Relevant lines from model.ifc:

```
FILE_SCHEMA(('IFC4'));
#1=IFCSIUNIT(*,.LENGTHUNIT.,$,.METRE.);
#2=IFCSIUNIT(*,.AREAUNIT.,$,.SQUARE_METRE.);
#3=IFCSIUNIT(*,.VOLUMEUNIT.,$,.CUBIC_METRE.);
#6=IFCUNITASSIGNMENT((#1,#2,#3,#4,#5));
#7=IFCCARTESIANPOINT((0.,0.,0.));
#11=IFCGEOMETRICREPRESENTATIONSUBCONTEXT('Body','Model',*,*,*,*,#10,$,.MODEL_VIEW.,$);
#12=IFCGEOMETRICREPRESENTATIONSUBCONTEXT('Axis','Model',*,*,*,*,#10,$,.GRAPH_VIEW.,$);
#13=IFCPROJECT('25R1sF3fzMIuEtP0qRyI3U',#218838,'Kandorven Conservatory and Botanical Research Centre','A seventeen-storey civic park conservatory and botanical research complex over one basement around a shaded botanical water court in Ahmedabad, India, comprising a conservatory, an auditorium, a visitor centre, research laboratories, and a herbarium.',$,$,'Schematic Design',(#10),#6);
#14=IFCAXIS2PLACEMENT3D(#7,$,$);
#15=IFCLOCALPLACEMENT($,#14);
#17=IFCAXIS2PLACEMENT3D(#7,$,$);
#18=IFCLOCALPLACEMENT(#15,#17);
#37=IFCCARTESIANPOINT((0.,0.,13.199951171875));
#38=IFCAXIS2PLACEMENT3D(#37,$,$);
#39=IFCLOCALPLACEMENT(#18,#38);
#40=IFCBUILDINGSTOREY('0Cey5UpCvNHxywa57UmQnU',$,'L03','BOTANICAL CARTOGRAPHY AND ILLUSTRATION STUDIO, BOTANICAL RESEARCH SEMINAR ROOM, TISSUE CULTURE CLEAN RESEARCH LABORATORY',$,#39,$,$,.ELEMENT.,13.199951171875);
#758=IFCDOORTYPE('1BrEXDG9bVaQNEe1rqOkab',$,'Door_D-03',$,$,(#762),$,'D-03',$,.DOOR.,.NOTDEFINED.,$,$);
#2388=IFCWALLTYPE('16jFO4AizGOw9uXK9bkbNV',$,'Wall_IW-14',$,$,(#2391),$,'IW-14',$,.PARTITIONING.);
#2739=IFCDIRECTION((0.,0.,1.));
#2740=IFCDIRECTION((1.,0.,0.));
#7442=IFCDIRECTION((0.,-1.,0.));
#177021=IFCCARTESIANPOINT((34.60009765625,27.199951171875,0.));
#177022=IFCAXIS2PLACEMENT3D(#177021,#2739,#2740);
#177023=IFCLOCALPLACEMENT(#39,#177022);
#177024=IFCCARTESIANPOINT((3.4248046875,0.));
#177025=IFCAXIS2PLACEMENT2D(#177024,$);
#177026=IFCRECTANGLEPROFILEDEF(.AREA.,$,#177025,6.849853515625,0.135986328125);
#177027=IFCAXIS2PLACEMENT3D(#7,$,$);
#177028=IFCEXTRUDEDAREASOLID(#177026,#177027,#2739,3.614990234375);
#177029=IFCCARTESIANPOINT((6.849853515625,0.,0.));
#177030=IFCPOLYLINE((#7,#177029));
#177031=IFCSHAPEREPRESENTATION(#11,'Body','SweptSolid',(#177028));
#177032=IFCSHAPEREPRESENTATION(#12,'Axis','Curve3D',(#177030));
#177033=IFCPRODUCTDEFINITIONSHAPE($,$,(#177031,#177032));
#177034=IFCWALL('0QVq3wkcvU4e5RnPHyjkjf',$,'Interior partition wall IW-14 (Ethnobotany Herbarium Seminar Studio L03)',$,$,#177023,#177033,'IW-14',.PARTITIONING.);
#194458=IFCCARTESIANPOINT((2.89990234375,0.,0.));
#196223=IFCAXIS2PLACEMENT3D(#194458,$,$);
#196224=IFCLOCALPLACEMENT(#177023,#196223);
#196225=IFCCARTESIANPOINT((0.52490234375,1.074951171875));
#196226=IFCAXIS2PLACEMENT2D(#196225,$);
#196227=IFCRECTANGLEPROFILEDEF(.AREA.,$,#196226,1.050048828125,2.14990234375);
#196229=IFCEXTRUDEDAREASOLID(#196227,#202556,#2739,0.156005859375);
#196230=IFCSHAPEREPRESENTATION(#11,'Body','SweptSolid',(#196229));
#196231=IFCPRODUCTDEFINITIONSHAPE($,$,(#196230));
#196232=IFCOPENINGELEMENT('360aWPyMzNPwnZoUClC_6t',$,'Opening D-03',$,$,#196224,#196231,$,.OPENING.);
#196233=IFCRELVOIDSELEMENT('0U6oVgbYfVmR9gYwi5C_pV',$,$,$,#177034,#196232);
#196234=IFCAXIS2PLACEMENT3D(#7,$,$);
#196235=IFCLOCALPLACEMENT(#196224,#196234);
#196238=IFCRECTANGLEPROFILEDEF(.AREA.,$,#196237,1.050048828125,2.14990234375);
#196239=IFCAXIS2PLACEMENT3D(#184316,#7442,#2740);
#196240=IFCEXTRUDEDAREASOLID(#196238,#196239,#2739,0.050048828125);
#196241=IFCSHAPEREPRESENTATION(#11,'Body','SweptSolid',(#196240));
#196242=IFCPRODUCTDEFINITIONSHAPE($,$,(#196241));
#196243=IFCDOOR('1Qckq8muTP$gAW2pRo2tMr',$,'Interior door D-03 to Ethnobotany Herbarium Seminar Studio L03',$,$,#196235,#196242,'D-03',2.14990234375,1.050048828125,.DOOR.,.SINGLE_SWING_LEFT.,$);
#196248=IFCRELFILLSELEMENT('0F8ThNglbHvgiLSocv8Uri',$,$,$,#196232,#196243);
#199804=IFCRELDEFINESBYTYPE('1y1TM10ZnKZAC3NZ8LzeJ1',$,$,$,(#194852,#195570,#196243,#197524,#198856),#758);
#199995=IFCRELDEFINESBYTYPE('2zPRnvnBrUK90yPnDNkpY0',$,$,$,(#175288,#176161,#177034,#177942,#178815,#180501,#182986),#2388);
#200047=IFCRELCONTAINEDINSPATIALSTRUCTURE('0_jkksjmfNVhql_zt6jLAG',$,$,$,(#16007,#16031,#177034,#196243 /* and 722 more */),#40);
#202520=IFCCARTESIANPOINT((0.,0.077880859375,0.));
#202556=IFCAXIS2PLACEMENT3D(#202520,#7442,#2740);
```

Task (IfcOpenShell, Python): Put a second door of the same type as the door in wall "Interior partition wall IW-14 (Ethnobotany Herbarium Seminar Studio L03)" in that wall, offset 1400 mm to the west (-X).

```python
import ifcopenshell
import ifcopenshell.api.feature
import ifcopenshell.api.geometry
import ifcopenshell.api.root
import ifcopenshell.geom
import ifcopenshell.util.element
import ifcopenshell.util.placement
import ifcopenshell.util.shape
import ifcopenshell.util.unit

model = ifcopenshell.open("model.ifc")
unit_scale = ifcopenshell.util.unit.calculate_unit_scale(model)
settings = ifcopenshell.geom.settings()


def volume(element):
    """Net volume in cubic metres, openings subtracted."""
    shape = ifcopenshell.geom.create_shape(settings, element)
    return ifcopenshell.util.shape.get_volume(shape.geometry)


door = model.by_guid("1Qckq8muTP$gAW2pRo2tMr")
opening = door.FillsVoids[0].RelatingOpeningElement
wall = opening.VoidsElements[0].RelatingBuildingElement
before = volume(wall)
shift = ifcopenshell.util.placement.get_local_placement(wall.ObjectPlacement)[:3, 0] * -1.4 / unit_scale

# copy_class copies the void relationship, type, container and properties, but no geometry.
new_opening = ifcopenshell.api.root.copy_class(model, product=opening)
new_opening.Representation = ifcopenshell.util.element.copy_deep(
    model, opening.Representation, exclude=["IfcGeometricRepresentationContext", "IfcRepresentationMap"]
)
new_door = ifcopenshell.api.root.copy_class(model, product=door)
new_door.Representation = ifcopenshell.util.element.copy_deep(
    model, door.Representation, exclude=["IfcGeometricRepresentationContext", "IfcRepresentationMap"]
)
new_door.Tag = None
ifcopenshell.api.feature.add_filling(model, opening=new_opening, element=new_door)

for old, new in ((opening, new_opening), (door, new_door)):
    matrix = ifcopenshell.util.placement.get_local_placement(old.ObjectPlacement)
    matrix[:3, 3] += shift
    ifcopenshell.api.geometry.edit_object_placement(model, product=new, matrix=matrix, is_si=False)

after = volume(wall)

print(f"wall volume {before:.3f} -> {after:.3f} m3")

model.write("model_edited.ifc")
```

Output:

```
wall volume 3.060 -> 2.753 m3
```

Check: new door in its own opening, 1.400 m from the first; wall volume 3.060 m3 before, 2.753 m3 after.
